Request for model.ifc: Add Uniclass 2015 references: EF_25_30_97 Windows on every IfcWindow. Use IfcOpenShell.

First a look at what the model holds.

```python
import ifcopenshell

model = ifcopenshell.open("model.ifc")
print(model.schema)
print("classifications:", [c.Name for c in model.by_type("IfcClassification")])
for ifc_class in ("IfcDoor", "IfcRoof", "IfcStair", "IfcWall", "IfcWindow"):
    print(ifc_class, len(model.by_type(ifc_class)))
```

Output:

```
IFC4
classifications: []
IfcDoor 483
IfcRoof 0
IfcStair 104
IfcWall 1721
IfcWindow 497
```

```python
import ifcopenshell
import ifcopenshell.api.classification

model = ifcopenshell.open("model.ifc")

system = ifcopenshell.api.classification.add_classification(model, classification="Uniclass 2015")

codes = {
    "IfcWindow": ("EF_25_30_97", "Windows"),
}
for ifc_class, (code, name) in codes.items():
    products = model.by_type(ifc_class)
    ifcopenshell.api.classification.add_reference(
        model, products=products, classification=system, identification=code, name=name
    )
    print(code, len(products))

model.write("model-out.ifc")
```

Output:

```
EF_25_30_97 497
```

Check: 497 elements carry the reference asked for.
